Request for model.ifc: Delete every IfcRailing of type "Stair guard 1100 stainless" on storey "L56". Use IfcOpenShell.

First a look at what the model holds.

```python
import ifcopenshell
import ifcopenshell.util.element

model = ifcopenshell.open("model.ifc")
print(model.schema)
storey = next(s for s in model.by_type("IfcBuildingStorey") if s.Name == "L56")
railings = [e for e in ifcopenshell.util.element.get_decomposition(storey) if e.is_a("IfcRailing")]
seen = {}
for e in railings:
    element_type = ifcopenshell.util.element.get_type(e)
    name = element_type.Name if element_type not in (None, e) else None
    seen[name] = seen.get(name, 0) + 1
for name, count in sorted(seen.items(), key=str):
    print(count, "x", name)
```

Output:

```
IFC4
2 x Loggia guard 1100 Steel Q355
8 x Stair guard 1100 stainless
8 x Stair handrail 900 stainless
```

```python
import ifcopenshell
import ifcopenshell.api.root
import ifcopenshell.util.element

model = ifcopenshell.open("model.ifc")

storey = next(s for s in model.by_type("IfcBuildingStorey") if s.Name == "L56")
railings = [e for e in ifcopenshell.util.element.get_decomposition(storey) if e.is_a("IfcRailing")]
targets = [e for e in railings if (t := ifcopenshell.util.element.get_type(e)) not in (None, e) and t.Name == "Stair guard 1100 stainless"]

for e in targets:
    ifcopenshell.api.root.remove_product(model, product=e)
print(len(targets), "removed")

model.write("model_rev.ifc")
```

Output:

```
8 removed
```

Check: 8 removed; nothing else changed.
